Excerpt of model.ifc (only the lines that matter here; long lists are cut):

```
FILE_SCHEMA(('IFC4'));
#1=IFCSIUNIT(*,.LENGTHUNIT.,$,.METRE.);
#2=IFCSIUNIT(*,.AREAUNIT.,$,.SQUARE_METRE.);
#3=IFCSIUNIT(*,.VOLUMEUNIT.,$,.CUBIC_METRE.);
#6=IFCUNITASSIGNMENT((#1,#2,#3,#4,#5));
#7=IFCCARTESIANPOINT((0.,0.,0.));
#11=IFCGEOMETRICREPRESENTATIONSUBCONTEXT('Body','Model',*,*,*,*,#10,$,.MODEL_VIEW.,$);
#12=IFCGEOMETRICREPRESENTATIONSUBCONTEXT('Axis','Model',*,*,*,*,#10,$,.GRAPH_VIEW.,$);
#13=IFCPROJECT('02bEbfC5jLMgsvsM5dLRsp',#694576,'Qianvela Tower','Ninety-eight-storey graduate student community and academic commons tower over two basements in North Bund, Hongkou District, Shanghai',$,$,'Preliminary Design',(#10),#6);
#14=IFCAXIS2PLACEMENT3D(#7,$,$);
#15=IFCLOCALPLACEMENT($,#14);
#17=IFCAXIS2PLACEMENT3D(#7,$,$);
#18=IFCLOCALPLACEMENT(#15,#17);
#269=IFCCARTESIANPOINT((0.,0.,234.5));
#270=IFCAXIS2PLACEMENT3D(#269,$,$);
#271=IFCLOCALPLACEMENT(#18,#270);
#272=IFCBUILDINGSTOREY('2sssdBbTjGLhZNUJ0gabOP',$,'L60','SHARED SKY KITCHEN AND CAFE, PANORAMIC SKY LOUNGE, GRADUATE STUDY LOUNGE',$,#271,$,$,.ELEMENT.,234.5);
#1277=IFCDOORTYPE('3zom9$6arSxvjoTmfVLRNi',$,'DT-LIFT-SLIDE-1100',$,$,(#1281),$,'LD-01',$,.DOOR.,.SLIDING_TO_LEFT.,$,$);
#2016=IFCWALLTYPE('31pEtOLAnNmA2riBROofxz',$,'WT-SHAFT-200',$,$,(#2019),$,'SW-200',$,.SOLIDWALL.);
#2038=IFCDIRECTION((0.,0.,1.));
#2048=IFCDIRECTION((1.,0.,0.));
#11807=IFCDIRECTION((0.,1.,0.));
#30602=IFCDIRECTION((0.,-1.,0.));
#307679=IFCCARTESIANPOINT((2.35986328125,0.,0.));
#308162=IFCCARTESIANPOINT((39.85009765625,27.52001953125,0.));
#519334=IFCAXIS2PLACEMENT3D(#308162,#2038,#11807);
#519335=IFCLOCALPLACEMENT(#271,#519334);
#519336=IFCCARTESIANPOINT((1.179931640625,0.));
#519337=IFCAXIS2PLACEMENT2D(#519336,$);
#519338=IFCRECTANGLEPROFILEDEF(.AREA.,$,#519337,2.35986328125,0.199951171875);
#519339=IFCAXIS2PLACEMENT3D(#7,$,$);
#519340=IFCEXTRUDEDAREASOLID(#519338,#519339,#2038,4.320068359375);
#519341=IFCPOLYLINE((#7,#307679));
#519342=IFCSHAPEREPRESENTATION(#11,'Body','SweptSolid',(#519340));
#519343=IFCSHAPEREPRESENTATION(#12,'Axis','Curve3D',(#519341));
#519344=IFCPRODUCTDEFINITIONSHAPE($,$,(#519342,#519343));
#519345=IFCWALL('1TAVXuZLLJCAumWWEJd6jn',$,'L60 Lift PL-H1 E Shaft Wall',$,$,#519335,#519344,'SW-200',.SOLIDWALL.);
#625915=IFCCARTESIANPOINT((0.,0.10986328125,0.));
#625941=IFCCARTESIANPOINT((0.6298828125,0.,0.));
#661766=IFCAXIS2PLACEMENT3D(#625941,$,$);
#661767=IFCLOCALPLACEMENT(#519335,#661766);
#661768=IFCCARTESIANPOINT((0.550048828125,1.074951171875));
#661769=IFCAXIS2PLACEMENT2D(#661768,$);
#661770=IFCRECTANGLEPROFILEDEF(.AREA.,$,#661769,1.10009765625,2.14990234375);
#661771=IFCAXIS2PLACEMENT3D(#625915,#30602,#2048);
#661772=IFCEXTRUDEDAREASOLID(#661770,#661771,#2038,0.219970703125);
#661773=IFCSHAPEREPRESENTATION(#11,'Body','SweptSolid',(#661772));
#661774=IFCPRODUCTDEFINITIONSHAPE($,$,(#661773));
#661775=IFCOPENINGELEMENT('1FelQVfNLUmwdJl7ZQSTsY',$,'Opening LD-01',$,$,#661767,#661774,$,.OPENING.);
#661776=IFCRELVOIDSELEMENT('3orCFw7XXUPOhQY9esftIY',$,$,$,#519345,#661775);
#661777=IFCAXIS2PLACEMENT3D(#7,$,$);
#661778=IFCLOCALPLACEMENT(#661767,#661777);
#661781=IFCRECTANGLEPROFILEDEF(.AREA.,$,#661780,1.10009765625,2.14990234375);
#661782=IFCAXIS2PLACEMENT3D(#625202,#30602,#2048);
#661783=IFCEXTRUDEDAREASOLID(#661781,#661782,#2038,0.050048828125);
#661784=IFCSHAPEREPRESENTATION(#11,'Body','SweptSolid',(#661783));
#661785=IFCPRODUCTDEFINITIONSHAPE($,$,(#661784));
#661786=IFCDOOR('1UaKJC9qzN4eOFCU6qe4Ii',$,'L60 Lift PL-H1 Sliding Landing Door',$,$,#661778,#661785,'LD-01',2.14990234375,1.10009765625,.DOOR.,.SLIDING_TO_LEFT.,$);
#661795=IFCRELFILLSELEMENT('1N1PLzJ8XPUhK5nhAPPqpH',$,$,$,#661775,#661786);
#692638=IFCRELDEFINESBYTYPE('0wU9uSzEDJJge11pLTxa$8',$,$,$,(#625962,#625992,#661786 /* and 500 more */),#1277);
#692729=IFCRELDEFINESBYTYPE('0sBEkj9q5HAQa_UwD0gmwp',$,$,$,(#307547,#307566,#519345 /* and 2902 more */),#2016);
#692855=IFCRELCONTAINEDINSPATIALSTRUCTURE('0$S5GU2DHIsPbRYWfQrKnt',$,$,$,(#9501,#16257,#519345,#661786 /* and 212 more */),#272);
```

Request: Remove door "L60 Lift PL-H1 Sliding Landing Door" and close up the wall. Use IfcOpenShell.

```python
import ifcopenshell
import ifcopenshell.api.feature
import ifcopenshell.api.root
import ifcopenshell.geom
import ifcopenshell.util.shape

model = ifcopenshell.open("model.ifc")
settings = ifcopenshell.geom.settings()


def volume(element):
    """Net volume in cubic metres, openings subtracted."""
    shape = ifcopenshell.geom.create_shape(settings, element)
    return ifcopenshell.util.shape.get_volume(shape.geometry)


door = model.by_guid("1UaKJC9qzN4eOFCU6qe4Ii")
opening = door.FillsVoids[0].RelatingOpeningElement
wall = opening.VoidsElements[0].RelatingBuildingElement
before = volume(wall)

ifcopenshell.api.root.remove_product(model, product=door)
ifcopenshell.api.feature.remove_feature(model, feature=opening)

after = volume(wall)

print(f"wall volume {before:.3f} -> {after:.3f} m3")

model.write("model_updated.ifc")
```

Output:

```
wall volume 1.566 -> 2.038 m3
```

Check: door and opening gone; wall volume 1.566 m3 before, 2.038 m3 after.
